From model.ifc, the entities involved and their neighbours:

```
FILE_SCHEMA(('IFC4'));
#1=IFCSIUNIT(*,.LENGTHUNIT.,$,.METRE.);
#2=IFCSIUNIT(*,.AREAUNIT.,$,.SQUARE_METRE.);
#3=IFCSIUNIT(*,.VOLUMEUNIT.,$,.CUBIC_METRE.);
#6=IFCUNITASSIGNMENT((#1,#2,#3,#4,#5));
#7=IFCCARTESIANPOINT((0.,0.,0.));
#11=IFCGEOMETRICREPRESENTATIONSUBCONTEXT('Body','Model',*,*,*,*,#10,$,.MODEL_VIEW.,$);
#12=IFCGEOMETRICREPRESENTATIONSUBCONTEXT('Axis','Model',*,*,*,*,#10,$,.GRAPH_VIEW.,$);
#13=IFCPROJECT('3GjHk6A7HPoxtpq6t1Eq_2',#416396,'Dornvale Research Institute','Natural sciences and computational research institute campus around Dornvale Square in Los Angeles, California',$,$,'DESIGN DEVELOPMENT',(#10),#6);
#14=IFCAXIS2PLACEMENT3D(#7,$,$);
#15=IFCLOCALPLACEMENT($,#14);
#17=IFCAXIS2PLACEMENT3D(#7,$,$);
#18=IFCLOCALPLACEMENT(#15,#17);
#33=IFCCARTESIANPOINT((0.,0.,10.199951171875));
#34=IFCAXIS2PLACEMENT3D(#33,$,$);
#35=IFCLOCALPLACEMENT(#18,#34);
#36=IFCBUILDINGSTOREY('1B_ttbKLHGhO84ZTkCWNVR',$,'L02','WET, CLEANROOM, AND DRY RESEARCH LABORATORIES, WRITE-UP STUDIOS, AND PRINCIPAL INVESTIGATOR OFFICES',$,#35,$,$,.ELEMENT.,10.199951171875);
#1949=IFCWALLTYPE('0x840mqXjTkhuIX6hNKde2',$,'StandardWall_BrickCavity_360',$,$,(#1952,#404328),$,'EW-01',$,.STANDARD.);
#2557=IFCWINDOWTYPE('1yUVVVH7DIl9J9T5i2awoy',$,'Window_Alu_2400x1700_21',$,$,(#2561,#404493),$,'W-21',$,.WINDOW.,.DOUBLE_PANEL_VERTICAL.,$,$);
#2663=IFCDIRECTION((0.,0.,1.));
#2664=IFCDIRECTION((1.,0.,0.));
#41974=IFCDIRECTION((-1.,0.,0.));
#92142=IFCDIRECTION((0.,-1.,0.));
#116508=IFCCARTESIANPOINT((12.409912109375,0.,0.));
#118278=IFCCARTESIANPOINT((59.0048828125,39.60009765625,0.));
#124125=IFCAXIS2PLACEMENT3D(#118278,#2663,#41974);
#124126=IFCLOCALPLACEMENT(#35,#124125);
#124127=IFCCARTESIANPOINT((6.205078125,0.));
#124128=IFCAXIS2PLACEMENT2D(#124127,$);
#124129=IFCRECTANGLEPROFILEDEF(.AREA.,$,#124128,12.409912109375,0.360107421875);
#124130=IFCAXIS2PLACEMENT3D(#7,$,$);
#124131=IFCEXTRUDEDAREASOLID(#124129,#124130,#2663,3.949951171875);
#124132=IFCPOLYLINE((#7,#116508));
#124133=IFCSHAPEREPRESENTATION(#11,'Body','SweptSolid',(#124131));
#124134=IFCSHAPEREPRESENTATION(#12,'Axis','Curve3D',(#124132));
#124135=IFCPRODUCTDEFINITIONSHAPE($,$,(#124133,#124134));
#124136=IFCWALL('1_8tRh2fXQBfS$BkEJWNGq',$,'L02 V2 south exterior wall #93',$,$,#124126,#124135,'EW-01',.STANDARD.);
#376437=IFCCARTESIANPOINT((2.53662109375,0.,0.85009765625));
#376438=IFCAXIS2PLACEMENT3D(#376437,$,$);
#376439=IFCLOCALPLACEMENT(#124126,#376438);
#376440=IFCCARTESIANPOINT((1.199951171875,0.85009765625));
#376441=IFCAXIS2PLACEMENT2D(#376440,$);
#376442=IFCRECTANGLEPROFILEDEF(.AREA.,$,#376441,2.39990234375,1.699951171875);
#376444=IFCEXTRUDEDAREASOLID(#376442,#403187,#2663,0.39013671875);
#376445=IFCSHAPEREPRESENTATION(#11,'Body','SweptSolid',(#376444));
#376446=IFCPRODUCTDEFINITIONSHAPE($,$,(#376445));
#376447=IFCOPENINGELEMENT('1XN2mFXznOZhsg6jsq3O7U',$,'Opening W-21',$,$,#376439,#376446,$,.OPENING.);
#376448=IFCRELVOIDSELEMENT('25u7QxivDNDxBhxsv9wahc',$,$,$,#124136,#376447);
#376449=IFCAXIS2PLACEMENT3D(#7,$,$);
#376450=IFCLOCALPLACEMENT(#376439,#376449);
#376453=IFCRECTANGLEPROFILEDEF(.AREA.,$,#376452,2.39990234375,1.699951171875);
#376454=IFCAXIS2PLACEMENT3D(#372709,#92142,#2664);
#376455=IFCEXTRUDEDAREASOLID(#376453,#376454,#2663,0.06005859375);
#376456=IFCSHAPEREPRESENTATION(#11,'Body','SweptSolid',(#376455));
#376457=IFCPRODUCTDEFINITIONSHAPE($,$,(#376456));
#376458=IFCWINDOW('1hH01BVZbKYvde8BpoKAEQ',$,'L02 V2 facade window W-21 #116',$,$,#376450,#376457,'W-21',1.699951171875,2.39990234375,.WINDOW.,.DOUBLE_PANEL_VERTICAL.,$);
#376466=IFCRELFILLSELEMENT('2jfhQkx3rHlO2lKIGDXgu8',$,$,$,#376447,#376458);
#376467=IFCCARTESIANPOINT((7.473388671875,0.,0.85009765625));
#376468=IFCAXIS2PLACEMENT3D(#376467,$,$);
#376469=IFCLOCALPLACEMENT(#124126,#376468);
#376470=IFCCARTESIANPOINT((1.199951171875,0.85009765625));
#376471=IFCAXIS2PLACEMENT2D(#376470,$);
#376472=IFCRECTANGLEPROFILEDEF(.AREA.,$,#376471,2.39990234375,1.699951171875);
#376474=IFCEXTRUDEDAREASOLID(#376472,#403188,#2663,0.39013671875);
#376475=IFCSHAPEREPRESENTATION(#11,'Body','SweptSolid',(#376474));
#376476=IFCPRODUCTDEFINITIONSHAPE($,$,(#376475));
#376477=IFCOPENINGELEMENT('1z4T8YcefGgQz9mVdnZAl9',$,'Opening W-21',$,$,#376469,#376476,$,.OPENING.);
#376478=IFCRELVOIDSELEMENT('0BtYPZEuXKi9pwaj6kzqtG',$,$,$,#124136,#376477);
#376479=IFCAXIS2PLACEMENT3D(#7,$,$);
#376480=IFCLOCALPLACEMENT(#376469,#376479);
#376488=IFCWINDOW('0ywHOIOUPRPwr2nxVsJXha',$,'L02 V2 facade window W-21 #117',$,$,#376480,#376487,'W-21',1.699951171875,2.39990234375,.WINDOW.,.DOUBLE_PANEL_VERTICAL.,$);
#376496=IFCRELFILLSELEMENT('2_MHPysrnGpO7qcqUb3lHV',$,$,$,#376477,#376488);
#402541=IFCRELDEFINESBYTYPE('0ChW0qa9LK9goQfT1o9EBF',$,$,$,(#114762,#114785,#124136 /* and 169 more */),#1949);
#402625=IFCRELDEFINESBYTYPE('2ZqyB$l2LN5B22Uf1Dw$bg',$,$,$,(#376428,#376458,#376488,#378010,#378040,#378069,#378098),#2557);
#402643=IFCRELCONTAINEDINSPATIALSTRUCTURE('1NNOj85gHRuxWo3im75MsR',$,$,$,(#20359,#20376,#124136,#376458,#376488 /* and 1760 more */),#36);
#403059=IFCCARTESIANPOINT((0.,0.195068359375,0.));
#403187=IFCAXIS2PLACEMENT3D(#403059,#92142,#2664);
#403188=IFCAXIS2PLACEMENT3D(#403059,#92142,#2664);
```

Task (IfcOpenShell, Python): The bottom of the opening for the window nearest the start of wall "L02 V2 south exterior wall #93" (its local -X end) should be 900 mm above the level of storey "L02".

```python
import numpy as np
import ifcopenshell
import ifcopenshell.api.geometry
import ifcopenshell.geom
import ifcopenshell.util.element
import ifcopenshell.util.placement
import ifcopenshell.util.shape
import ifcopenshell.util.unit

model = ifcopenshell.open("model.ifc")
unit_scale = ifcopenshell.util.unit.calculate_unit_scale(model)

window = model.by_id(376458)
opening = window.FillsVoids[0].RelatingOpeningElement
storey = ifcopenshell.util.element.get_container(window, ifc_class="IfcBuildingStorey")
level = ifcopenshell.util.placement.get_local_placement(storey.ObjectPlacement)[2, 3]

# The opening's origin need not be at the sill, so measure its lowest point.
shape = ifcopenshell.geom.create_shape(ifcopenshell.geom.settings(), opening)
bottom = ifcopenshell.util.shape.get_shape_bottom_elevation(shape, shape.geometry) / unit_scale
dz = level + 0.9 / unit_scale - bottom

shift = np.array([0.0, 0.0, dz])
# The window is placed relative to its opening, so it follows when the opening moves.
matrix = ifcopenshell.util.placement.get_local_placement(opening.ObjectPlacement)
matrix[:3, 3] += shift
ifcopenshell.api.geometry.edit_object_placement(
    model, product=opening, matrix=matrix, is_si=False, should_transform_children=True
)

print(f"moved by {dz * unit_scale:+.3f} m")

model.write("model-out.ifc")
```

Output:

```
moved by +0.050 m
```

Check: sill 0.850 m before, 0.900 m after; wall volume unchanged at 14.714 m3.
